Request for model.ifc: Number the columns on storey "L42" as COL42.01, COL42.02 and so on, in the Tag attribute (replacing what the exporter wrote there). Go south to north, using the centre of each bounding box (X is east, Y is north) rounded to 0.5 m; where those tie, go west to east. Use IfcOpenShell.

First a look at what the model holds.

```python
import ifcopenshell
import ifcopenshell.util.element
import ifcopenshell.util.placement

model = ifcopenshell.open("model.ifc")
print(model.schema)
storey = next(s for s in model.by_type("IfcBuildingStorey") if s.Name == "L42")
columns = [e for e in ifcopenshell.util.element.get_decomposition(storey) if e.is_a("IfcColumn")]
for e in sorted(columns, key=lambda e: e.id()):
    origin = ifcopenshell.util.placement.get_local_placement(e.ObjectPlacement)[:3, 3]
    print(e.id(), e.Tag, e.Name, origin.round(2) + 0.0, sep=" | ")
```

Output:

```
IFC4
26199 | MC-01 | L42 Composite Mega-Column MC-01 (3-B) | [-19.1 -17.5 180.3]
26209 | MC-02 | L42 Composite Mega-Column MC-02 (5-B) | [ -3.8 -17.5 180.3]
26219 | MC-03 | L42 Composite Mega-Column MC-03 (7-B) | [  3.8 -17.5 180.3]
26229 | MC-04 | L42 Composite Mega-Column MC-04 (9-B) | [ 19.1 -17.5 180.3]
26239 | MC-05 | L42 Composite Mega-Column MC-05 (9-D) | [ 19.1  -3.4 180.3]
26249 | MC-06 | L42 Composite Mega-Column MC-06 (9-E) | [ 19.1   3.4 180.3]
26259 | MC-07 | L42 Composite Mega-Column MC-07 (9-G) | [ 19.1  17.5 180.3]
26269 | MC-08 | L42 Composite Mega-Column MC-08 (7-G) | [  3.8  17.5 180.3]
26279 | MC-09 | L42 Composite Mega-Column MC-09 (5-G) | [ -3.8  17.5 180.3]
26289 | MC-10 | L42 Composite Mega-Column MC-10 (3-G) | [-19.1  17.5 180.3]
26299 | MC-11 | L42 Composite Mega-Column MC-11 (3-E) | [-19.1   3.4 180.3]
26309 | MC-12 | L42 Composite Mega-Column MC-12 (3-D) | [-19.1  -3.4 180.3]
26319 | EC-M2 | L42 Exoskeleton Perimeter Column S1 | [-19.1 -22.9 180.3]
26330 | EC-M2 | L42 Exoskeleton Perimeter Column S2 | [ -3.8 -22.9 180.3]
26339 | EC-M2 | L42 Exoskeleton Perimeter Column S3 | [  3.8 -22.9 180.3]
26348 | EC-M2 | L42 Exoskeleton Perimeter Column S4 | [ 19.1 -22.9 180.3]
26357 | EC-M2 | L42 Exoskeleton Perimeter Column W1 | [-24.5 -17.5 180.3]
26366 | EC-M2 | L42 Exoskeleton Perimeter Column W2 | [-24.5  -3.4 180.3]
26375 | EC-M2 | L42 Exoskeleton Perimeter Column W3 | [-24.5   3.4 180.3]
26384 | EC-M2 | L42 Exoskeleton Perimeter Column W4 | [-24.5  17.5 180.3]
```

```python
import ifcopenshell
import ifcopenshell.geom
import ifcopenshell.util.element
import ifcopenshell.util.shape

model = ifcopenshell.open("model.ifc")
settings = ifcopenshell.geom.settings()
settings.set("use-world-coords", True)


def centre(element):
    shape = ifcopenshell.geom.create_shape(settings, element)
    return ifcopenshell.util.shape.get_bbox_centroid(shape.geometry)


storey = next(s for s in model.by_type("IfcBuildingStorey") if s.Name == "L42")
columns = [e for e in ifcopenshell.util.element.get_decomposition(storey) if e.is_a("IfcColumn")]

# Insertion points can sit at a corner or the storey origin, so sort by the geometry (in metres).
centres = {e: centre(e) for e in columns}
columns.sort(key=lambda e: (round(centres[e][1] / 0.5), centres[e][0]))

for i, e in enumerate(columns, start=1):
    number = f"COL42.{i:02d}"
    e.Tag = number
    print(e.id(), number)

model.write("model_edited.ifc")
```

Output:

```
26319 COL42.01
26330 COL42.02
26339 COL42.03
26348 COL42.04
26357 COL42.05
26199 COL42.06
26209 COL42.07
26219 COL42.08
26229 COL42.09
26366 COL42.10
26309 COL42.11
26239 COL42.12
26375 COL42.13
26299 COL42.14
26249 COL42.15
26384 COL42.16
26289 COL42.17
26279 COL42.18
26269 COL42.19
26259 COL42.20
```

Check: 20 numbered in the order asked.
